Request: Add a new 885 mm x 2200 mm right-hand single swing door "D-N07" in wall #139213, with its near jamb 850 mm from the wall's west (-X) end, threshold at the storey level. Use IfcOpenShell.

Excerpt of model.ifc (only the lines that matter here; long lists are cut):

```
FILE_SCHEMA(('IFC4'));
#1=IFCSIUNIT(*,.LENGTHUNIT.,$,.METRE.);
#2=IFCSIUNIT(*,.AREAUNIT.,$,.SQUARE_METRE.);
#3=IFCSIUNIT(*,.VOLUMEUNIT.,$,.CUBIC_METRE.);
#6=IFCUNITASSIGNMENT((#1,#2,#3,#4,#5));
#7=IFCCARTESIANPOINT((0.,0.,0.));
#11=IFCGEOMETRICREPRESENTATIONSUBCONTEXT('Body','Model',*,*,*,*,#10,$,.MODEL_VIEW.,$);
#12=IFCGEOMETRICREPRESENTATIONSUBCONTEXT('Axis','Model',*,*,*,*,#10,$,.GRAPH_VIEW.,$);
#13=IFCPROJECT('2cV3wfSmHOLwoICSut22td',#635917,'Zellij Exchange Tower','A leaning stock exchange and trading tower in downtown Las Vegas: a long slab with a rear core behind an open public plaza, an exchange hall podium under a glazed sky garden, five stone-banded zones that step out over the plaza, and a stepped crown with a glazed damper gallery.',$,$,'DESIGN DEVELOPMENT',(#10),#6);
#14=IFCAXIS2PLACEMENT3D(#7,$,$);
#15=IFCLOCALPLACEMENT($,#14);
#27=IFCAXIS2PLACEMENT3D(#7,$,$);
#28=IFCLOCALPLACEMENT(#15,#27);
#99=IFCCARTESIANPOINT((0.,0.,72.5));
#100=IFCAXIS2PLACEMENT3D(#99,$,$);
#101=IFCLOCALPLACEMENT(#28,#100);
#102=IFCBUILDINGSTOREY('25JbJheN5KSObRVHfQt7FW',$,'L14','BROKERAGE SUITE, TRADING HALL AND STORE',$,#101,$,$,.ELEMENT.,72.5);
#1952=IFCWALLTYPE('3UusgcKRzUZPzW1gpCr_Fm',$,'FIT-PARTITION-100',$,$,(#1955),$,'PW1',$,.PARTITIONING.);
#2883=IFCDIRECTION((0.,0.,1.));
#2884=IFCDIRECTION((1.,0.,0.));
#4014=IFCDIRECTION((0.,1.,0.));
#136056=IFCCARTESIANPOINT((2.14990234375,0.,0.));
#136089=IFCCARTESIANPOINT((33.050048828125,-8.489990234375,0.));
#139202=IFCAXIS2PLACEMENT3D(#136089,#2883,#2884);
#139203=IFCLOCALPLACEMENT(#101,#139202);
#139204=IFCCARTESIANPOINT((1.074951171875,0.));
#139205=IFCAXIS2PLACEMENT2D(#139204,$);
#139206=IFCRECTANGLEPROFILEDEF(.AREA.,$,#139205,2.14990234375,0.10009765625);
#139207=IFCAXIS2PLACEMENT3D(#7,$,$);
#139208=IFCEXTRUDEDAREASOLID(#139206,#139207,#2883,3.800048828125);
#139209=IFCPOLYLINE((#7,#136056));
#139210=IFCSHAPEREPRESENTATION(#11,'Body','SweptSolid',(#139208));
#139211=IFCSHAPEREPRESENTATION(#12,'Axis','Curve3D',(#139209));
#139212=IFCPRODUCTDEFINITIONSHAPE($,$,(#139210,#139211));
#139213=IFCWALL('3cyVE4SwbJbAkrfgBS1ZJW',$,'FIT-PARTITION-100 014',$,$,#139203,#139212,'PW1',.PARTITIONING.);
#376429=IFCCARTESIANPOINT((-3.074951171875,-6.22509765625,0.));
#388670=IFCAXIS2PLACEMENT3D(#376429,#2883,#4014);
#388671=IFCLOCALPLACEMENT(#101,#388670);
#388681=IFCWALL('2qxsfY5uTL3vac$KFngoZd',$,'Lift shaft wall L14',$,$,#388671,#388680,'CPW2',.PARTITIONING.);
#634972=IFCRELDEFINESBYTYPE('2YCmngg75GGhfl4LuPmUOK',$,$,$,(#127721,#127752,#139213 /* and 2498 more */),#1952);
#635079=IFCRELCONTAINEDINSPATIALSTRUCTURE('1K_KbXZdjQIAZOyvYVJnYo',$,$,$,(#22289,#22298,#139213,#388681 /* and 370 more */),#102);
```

```python
import numpy as np
import ifcopenshell
import ifcopenshell.api.feature
import ifcopenshell.api.geometry
import ifcopenshell.api.root
import ifcopenshell.api.spatial
import ifcopenshell.geom
import ifcopenshell.util.element
import ifcopenshell.util.placement
import ifcopenshell.util.representation
import ifcopenshell.util.shape
import ifcopenshell.util.unit

model = ifcopenshell.open("model.ifc")
unit_scale = ifcopenshell.util.unit.calculate_unit_scale(model)
settings = ifcopenshell.geom.settings()


def volume(element):
    """Net volume in cubic metres, openings subtracted."""
    shape = ifcopenshell.geom.create_shape(settings, element)
    return ifcopenshell.util.shape.get_volume(shape.geometry)


wall = model.by_guid("3cyVE4SwbJbAkrfgBS1ZJW")
storey = ifcopenshell.util.element.get_container(wall, ifc_class="IfcBuildingStorey")
context = ifcopenshell.util.representation.get_context(model, "Model", "Body", "MODEL_VIEW")
before = volume(wall)

width, height, from_end, sill = 0.885, 2.2, 0.85, 0.0  # metres

# The wall runs along its own X axis, and the end named is its -X end.
wall_shape = ifcopenshell.geom.create_shape(settings, wall)
x, y, z = ifcopenshell.util.shape.get_vertices(wall_shape.geometry).T
start = x.min() + from_end
face, thickness = float(y.min()), float(y.max() - y.min())
wall_matrix = ifcopenshell.util.placement.get_local_placement(wall.ObjectPlacement)
level = ifcopenshell.util.placement.get_local_placement(storey.ObjectPlacement)[2, 3]


def in_wall(x, y):
    """Placement at x, y metres in the wall's axes, at sill height."""
    matrix = wall_matrix.copy()
    matrix[:, 3] = wall_matrix @ np.array([x / unit_scale, y / unit_scale, 0.0, 1.0])
    matrix[2, 3] = level + sill / unit_scale
    return matrix


# Opening: a box that overshoots both wall faces by 50 mm.
opening = ifcopenshell.api.root.create_entity(model, ifc_class="IfcOpeningElement", predefined_type="OPENING")
box = ifcopenshell.api.geometry.add_wall_representation(
    model, context=context, length=width, height=height, thickness=thickness + 0.1
)
ifcopenshell.api.geometry.assign_representation(model, product=opening, representation=box)
ifcopenshell.api.geometry.edit_object_placement(model, product=opening, matrix=in_wall(start, face - 0.05), is_si=False)
ifcopenshell.api.feature.add_feature(model, feature=opening, element=wall)

door = ifcopenshell.api.root.create_entity(model, ifc_class="IfcDoor", name="D-N07", predefined_type="DOOR")
door.OverallWidth, door.OverallHeight = width / unit_scale, height / unit_scale
door.OperationType = "SINGLE_SWING_RIGHT"
body = ifcopenshell.api.geometry.add_door_representation(
    model,
    context=context,
    overall_width=door.OverallWidth,
    overall_height=door.OverallHeight,
    operation_type="SINGLE_SWING_RIGHT",
    lining_properties={"LiningDepth": thickness / unit_scale, "ThresholdDepth": thickness / unit_scale},
)
ifcopenshell.api.geometry.assign_representation(model, product=door, representation=body)
ifcopenshell.api.spatial.assign_container(model, products=[door], relating_structure=storey)
ifcopenshell.api.feature.add_filling(model, opening=opening, element=door)

# The lining spans the wall, so the door starts at the wall face.
ifcopenshell.api.geometry.edit_object_placement(model, product=door, matrix=in_wall(start, face), is_si=False)

after = volume(wall)

print(f"wall volume {before:.3f} -> {after:.3f} m3")

model.write("model_updated.ifc")
```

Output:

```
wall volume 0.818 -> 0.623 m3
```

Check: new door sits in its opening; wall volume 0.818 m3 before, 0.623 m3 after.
